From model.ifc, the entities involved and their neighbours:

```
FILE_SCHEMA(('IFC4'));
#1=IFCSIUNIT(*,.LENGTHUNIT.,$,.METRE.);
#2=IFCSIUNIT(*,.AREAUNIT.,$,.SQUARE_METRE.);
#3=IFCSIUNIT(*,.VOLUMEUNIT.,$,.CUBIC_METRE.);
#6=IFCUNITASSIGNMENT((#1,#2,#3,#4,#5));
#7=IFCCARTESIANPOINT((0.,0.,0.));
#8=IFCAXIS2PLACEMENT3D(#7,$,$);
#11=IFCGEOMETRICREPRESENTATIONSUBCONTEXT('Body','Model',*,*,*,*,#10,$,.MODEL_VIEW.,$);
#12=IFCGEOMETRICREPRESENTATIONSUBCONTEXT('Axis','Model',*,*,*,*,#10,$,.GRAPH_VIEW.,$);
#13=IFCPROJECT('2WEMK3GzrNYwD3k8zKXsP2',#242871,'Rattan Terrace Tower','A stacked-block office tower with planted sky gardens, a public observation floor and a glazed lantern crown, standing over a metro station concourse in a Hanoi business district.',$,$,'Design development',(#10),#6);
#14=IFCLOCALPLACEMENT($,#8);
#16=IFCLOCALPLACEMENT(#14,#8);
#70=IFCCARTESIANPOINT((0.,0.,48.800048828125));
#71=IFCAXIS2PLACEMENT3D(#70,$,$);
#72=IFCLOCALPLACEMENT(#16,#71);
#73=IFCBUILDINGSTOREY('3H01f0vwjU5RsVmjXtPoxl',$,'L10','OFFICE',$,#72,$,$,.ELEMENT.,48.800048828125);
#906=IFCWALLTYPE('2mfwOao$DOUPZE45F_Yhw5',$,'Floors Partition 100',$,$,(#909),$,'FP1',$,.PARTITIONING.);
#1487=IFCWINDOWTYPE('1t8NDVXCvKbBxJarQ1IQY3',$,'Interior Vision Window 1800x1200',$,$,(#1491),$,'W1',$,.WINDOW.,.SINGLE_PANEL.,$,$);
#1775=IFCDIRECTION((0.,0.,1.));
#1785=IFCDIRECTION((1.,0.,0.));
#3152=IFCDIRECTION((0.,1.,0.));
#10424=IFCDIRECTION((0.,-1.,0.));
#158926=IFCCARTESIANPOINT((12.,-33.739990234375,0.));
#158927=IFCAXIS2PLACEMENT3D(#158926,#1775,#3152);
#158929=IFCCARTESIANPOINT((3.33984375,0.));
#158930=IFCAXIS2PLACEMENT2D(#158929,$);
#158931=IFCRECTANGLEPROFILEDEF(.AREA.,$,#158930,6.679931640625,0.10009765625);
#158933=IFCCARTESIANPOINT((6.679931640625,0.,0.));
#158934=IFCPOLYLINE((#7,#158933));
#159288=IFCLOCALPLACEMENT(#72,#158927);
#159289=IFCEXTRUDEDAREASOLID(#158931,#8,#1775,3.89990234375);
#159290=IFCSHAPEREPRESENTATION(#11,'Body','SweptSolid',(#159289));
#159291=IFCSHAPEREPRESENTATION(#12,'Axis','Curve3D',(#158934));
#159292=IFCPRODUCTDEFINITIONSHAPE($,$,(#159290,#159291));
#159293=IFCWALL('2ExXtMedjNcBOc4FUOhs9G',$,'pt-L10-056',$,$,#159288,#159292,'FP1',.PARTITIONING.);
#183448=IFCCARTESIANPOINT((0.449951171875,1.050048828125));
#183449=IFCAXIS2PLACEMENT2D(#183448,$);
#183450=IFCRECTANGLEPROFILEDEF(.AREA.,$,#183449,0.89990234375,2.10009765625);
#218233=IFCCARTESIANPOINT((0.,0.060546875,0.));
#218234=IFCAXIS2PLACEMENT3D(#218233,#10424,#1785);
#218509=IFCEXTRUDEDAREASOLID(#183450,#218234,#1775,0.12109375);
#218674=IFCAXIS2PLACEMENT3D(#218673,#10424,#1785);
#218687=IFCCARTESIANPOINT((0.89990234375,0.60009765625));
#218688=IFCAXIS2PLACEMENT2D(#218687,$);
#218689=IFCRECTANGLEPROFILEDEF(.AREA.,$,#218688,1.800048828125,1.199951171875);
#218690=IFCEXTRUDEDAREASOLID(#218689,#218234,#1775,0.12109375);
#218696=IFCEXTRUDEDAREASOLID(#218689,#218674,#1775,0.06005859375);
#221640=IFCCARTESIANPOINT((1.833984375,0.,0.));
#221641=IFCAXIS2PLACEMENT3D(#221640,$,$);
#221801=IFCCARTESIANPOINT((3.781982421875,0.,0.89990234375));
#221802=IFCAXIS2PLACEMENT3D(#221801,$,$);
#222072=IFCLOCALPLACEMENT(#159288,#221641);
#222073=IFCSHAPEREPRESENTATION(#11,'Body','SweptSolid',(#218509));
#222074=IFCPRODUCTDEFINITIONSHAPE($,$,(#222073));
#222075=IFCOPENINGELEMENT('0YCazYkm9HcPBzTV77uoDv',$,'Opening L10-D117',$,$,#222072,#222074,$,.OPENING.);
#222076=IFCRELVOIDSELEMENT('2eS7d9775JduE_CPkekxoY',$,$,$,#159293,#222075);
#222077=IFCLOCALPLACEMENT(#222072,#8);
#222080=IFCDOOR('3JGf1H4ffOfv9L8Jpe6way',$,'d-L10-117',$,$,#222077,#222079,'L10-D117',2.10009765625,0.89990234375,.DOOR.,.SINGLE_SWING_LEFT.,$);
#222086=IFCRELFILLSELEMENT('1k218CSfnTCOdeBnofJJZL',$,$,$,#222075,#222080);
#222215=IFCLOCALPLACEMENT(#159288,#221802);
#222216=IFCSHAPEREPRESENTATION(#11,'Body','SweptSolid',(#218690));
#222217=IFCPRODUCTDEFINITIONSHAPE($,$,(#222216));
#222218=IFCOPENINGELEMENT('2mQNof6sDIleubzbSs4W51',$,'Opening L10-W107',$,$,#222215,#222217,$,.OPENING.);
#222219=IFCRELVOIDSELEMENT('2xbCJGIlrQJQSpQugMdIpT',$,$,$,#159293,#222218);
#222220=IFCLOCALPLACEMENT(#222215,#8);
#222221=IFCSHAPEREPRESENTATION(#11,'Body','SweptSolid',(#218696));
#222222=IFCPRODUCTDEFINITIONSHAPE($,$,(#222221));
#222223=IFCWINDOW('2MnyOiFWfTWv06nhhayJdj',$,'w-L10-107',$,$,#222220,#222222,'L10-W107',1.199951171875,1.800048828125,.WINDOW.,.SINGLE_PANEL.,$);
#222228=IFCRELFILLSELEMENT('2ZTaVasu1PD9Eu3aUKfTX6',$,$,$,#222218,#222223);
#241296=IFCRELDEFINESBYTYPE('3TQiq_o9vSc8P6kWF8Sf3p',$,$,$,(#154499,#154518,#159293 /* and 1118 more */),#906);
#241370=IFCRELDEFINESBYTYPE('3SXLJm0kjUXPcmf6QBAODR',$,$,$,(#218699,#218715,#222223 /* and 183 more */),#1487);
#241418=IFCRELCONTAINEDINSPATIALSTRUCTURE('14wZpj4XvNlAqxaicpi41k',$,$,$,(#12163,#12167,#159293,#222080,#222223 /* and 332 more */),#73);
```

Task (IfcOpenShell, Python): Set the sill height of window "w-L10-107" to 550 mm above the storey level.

```python
import numpy as np
import ifcopenshell
import ifcopenshell.api.geometry
import ifcopenshell.geom
import ifcopenshell.util.element
import ifcopenshell.util.placement
import ifcopenshell.util.shape
import ifcopenshell.util.unit

model = ifcopenshell.open("model.ifc")
unit_scale = ifcopenshell.util.unit.calculate_unit_scale(model)

window = model.by_guid("2MnyOiFWfTWv06nhhayJdj")
opening = window.FillsVoids[0].RelatingOpeningElement
storey = ifcopenshell.util.element.get_container(window, ifc_class="IfcBuildingStorey")
level = ifcopenshell.util.placement.get_local_placement(storey.ObjectPlacement)[2, 3]

# The opening's origin need not be at the sill, so measure its lowest point.
shape = ifcopenshell.geom.create_shape(ifcopenshell.geom.settings(), opening)
bottom = ifcopenshell.util.shape.get_shape_bottom_elevation(shape, shape.geometry) / unit_scale
dz = level + 0.55 / unit_scale - bottom

shift = np.array([0.0, 0.0, dz])
# The window is placed relative to its opening, so it follows when the opening moves.
matrix = ifcopenshell.util.placement.get_local_placement(opening.ObjectPlacement)
matrix[:3, 3] += shift
ifcopenshell.api.geometry.edit_object_placement(
    model, product=opening, matrix=matrix, is_si=False, should_transform_children=True
)

print(f"moved by {dz * unit_scale:+.3f} m")

model.write("model_edited.ifc")
```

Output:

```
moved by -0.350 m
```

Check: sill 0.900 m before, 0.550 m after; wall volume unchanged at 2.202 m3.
